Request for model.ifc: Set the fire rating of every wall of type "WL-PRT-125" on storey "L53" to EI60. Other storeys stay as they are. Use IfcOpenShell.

First a look at what the model holds.

```python
import ifcopenshell
import ifcopenshell.util.element

model = ifcopenshell.open("model.ifc")
print(model.schema)
storey = next(s for s in model.by_type("IfcBuildingStorey") if s.Name == "L53")
walls = [e for e in ifcopenshell.util.element.get_decomposition(storey) if e.is_a("IfcWall")]
seen = {}
for e in walls:
    element_type = ifcopenshell.util.element.get_type(e)
    key = (element_type.Name if element_type != e and element_type else None, ifcopenshell.util.element.get_pset(e, "Pset_WallCommon", "FireRating"))
    seen[key] = seen.get(key, 0) + 1
for (name, value), count in sorted(seen.items(), key=str):
    print(count, "x", name, "|", value)
```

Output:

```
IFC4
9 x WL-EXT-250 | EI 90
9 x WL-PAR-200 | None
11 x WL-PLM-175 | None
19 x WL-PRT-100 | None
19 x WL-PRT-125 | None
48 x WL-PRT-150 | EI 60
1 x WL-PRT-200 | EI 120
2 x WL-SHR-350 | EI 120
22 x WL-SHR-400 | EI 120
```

```python
import ifcopenshell
import ifcopenshell.api.pset
import ifcopenshell.util.element

model = ifcopenshell.open("model.ifc")

storey = next(s for s in model.by_type("IfcBuildingStorey") if s.Name == "L53")
walls = [e for e in ifcopenshell.util.element.get_decomposition(storey) if e.is_a("IfcWall")]

count = 0
for e in walls:
    element_type = ifcopenshell.util.element.get_type(e)
    if element_type in (None, e) or element_type.Name != "WL-PRT-125":
        continue
    # add_pset returns the element's existing set when there is one.
    pset = ifcopenshell.api.pset.add_pset(model, product=e, name="Pset_WallCommon")
    ifcopenshell.api.pset.edit_pset(model, pset=pset, properties={"FireRating": "EI60"})
    count += 1

print(count, "walls updated")

model.write("model_rev.ifc")
```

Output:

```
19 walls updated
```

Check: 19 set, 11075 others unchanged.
